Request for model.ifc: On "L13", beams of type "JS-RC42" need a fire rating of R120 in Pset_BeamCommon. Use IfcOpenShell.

First a look at what the model holds.

```python
import ifcopenshell
import ifcopenshell.util.element

model = ifcopenshell.open("model.ifc")
print(model.schema)
storey = next(s for s in model.by_type("IfcBuildingStorey") if s.Name == "L13")
beams = [e for e in ifcopenshell.util.element.get_decomposition(storey) if e.is_a("IfcBeam")]
seen = {}
for e in beams:
    element_type = ifcopenshell.util.element.get_type(e)
    key = (element_type.Name if element_type != e and element_type else None, ifcopenshell.util.element.get_pset(e, "Pset_BeamCommon", "FireRating"))
    seen[key] = seen.get(key, 0) + 1
for (name, value), count in sorted(seen.items(), key=str):
    print(count, "x", name, "|", value)
```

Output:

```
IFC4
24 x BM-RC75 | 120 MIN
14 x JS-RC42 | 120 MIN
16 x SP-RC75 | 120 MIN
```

```python
import ifcopenshell
import ifcopenshell.api.pset
import ifcopenshell.util.element

model = ifcopenshell.open("model.ifc")

storey = next(s for s in model.by_type("IfcBuildingStorey") if s.Name == "L13")
beams = [e for e in ifcopenshell.util.element.get_decomposition(storey) if e.is_a("IfcBeam")]

count = 0
for e in beams:
    element_type = ifcopenshell.util.element.get_type(e)
    if element_type in (None, e) or element_type.Name != "JS-RC42":
        continue
    # add_pset returns the element's existing set when there is one.
    pset = ifcopenshell.api.pset.add_pset(model, product=e, name="Pset_BeamCommon")
    ifcopenshell.api.pset.edit_pset(model, pset=pset, properties={"FireRating": "R120"})
    count += 1

print(count, "beams updated")

model.write("model_edited.ifc")
```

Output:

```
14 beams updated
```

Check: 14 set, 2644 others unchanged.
